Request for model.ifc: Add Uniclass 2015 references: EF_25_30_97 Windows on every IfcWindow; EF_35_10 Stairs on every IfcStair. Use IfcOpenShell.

First a look at what the model holds.

```python
import ifcopenshell

model = ifcopenshell.open("model.ifc")
print(model.schema)
print("classifications:", [c.Name for c in model.by_type("IfcClassification")])
for ifc_class in ("IfcDoor", "IfcRoof", "IfcStair", "IfcWall", "IfcWindow"):
    print(ifc_class, len(model.by_type(ifc_class)))
```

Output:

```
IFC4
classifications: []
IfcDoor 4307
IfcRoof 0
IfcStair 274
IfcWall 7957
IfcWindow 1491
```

```python
import ifcopenshell
import ifcopenshell.api.classification

model = ifcopenshell.open("model.ifc")

system = ifcopenshell.api.classification.add_classification(model, classification="Uniclass 2015")

codes = {
    "IfcWindow": ("EF_25_30_97", "Windows"),
    "IfcStair": ("EF_35_10", "Stairs"),
}
for ifc_class, (code, name) in codes.items():
    products = model.by_type(ifc_class)
    ifcopenshell.api.classification.add_reference(
        model, products=products, classification=system, identification=code, name=name
    )
    print(code, len(products))

model.write("model_edited.ifc")
```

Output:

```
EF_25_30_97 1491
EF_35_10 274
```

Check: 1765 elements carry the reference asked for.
